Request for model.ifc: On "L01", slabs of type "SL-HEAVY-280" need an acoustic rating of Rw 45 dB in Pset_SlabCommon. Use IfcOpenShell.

First a look at what the model holds.

```python
import ifcopenshell
import ifcopenshell.util.element

model = ifcopenshell.open("model.ifc")
print(model.schema)
storey = next(s for s in model.by_type("IfcBuildingStorey") if s.Name == "L01")
slabs = [e for e in ifcopenshell.util.element.get_decomposition(storey) if e.is_a("IfcSlab")]
seen = {}
for e in slabs:
    element_type = ifcopenshell.util.element.get_type(e)
    key = (element_type.Name if element_type != e and element_type else None, ifcopenshell.util.element.get_pset(e, "Pset_SlabCommon", "AcousticRating"))
    seen[key] = seen.get(key, 0) + 1
for (name, value), count in sorted(seen.items(), key=str):
    print(count, "x", name, "|", value)
```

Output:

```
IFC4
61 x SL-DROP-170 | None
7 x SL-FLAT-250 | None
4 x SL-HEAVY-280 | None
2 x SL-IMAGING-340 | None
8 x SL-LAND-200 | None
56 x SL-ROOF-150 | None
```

```python
import ifcopenshell
import ifcopenshell.api.pset
import ifcopenshell.util.element

model = ifcopenshell.open("model.ifc")

storey = next(s for s in model.by_type("IfcBuildingStorey") if s.Name == "L01")
slabs = [e for e in ifcopenshell.util.element.get_decomposition(storey) if e.is_a("IfcSlab")]

count = 0
for e in slabs:
    element_type = ifcopenshell.util.element.get_type(e)
    if element_type in (None, e) or element_type.Name != "SL-HEAVY-280":
        continue
    # add_pset returns the element's existing set when there is one.
    pset = ifcopenshell.api.pset.add_pset(model, product=e, name="Pset_SlabCommon")
    ifcopenshell.api.pset.edit_pset(model, pset=pset, properties={"AcousticRating": "Rw 45 dB"})
    count += 1

print(count, "slabs updated")

model.write("model_edited.ifc")
```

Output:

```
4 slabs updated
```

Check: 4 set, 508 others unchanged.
